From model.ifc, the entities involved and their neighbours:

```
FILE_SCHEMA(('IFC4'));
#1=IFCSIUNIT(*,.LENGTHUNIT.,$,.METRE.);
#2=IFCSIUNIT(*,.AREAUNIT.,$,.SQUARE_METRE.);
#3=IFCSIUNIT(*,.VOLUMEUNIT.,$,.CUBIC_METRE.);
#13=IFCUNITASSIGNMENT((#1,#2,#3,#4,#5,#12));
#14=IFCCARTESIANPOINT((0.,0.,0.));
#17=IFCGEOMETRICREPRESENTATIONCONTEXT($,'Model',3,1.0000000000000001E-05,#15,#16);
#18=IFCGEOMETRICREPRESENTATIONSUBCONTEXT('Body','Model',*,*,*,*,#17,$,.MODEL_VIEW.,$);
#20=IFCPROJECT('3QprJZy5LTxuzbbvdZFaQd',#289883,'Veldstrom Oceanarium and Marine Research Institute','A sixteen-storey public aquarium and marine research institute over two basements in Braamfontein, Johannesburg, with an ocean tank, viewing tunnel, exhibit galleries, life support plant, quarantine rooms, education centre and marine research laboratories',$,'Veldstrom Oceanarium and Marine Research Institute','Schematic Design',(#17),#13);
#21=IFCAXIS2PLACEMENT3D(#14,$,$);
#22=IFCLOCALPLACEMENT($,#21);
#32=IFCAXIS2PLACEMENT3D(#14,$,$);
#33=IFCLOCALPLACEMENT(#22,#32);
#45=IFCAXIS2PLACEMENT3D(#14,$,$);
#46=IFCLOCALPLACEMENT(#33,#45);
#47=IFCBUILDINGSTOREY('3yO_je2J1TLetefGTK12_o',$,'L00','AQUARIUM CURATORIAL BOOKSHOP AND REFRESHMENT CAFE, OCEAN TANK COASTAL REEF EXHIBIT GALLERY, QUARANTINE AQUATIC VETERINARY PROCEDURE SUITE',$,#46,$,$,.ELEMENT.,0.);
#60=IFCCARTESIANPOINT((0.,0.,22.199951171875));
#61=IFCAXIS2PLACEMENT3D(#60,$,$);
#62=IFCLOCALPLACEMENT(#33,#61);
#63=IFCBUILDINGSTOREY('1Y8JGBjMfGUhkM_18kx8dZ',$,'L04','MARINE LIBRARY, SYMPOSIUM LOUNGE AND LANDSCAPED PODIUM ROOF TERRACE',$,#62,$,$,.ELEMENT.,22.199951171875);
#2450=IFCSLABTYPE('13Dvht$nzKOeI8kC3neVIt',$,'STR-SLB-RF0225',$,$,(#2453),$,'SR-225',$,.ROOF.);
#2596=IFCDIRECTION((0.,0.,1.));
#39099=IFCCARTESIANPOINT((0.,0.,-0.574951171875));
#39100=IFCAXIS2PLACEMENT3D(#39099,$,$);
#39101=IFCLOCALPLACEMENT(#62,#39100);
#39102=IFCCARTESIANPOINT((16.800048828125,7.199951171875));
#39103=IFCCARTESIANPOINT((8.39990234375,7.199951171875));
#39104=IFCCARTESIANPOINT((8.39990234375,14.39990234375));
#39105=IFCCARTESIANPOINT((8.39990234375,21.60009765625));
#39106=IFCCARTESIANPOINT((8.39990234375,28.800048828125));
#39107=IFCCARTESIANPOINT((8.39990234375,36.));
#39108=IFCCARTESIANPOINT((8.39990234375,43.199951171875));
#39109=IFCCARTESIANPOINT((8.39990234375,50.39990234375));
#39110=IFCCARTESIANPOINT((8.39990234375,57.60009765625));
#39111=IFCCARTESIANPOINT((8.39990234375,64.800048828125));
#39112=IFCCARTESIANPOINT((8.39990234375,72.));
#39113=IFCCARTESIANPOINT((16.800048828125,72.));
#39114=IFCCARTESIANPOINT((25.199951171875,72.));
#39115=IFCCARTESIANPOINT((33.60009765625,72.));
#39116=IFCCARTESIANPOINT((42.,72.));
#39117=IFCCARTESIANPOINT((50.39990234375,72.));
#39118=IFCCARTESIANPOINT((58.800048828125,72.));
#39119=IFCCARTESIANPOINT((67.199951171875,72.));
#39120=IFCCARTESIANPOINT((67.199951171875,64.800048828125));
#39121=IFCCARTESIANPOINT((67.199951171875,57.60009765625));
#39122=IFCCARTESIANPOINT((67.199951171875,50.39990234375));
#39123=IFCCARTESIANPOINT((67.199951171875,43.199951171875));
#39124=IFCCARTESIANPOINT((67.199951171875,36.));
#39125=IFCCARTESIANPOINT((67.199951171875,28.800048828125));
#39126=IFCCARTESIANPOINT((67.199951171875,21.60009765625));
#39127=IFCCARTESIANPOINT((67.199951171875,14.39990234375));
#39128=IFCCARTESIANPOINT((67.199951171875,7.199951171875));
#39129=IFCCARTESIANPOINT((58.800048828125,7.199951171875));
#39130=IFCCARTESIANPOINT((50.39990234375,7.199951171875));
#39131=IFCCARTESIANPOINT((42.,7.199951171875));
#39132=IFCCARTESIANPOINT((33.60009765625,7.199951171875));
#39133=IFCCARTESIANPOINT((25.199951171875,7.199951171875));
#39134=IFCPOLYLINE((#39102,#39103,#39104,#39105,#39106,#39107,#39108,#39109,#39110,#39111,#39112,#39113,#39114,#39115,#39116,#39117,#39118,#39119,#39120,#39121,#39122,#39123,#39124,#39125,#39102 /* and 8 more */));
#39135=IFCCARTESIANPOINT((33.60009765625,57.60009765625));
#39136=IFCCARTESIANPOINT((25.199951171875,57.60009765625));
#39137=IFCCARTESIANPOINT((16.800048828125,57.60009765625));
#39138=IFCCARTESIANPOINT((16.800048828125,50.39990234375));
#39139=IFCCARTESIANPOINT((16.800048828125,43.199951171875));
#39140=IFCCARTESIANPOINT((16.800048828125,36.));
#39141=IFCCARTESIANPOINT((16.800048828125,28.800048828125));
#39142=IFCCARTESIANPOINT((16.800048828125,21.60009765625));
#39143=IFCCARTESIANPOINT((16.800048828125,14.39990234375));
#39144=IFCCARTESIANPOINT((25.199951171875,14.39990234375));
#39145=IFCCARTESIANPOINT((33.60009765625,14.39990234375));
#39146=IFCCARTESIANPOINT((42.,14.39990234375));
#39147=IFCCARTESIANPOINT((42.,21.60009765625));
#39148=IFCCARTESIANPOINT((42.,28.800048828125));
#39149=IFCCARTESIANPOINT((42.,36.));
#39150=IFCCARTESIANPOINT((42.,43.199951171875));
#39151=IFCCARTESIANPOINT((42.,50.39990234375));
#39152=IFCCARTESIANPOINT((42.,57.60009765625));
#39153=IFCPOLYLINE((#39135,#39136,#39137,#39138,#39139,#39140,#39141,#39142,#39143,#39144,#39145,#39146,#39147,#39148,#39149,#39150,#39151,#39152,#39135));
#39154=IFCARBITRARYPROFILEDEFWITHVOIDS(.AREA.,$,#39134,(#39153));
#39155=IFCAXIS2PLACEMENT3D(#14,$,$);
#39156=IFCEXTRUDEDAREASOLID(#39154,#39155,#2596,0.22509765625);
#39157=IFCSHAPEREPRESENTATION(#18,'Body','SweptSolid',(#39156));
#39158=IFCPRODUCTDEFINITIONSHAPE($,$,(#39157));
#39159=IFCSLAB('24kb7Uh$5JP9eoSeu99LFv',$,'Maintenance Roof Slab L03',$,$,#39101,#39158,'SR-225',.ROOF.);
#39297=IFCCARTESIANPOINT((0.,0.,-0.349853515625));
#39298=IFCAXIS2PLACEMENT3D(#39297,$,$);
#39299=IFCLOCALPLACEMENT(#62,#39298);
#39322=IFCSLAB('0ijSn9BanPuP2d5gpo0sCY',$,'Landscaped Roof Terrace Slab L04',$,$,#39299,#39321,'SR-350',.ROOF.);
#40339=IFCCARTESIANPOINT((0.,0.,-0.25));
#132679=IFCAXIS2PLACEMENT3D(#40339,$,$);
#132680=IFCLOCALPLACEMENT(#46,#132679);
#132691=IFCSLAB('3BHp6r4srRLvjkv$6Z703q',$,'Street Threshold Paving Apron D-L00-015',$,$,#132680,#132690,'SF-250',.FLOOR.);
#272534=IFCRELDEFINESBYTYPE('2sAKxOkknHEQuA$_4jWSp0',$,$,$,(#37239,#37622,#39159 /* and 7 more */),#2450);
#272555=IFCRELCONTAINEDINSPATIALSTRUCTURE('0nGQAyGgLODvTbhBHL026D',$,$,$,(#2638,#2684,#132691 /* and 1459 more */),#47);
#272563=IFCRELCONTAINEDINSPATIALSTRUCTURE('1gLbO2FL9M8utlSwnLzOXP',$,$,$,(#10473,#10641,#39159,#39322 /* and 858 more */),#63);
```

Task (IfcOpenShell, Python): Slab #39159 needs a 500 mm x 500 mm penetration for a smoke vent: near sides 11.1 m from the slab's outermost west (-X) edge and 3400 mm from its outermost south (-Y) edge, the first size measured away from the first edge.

```python
import numpy as np
import ifcopenshell
import ifcopenshell.api.feature
import ifcopenshell.api.geometry
import ifcopenshell.api.root
import ifcopenshell.geom
import ifcopenshell.util.placement
import ifcopenshell.util.representation
import ifcopenshell.util.shape
import ifcopenshell.util.unit

model = ifcopenshell.open("model.ifc")
unit_scale = ifcopenshell.util.unit.calculate_unit_scale(model)
settings = ifcopenshell.geom.settings()


def volume(element):
    """Net volume in cubic metres, openings subtracted."""
    shape = ifcopenshell.geom.create_shape(settings, element)
    return ifcopenshell.util.shape.get_volume(shape.geometry)


slab = model.by_guid("24kb7Uh$5JP9eoSeu99LFv")
before = volume(slab)

# Extent in the slab's own axes, in metres. The edges named are its -X and -Y sides.
slab_shape = ifcopenshell.geom.create_shape(settings, slab)
vertices = ifcopenshell.util.shape.get_vertices(slab_shape.geometry)
x_min, y_min, bottom = vertices.min(axis=0)
top = vertices[:, 2].max()

opening = ifcopenshell.api.root.create_entity(model, ifc_class="IfcOpeningElement", name="Smoke vent opening", predefined_type="OPENING")
context = ifcopenshell.util.representation.get_context(model, "Model", "Body", "MODEL_VIEW")
width, depth = 0.5, 0.5
outline = [(0.0, 0.0), (width, 0.0), (width, depth), (0.0, depth), (0.0, 0.0)]
# Overshoot both faces by 50 mm so the cut is clean.
shape = ifcopenshell.api.geometry.add_slab_representation(
    model, context=context, depth=top - bottom + 0.1, polyline=outline
)
ifcopenshell.api.geometry.assign_representation(model, product=opening, representation=shape)

matrix = ifcopenshell.util.placement.get_local_placement(slab.ObjectPlacement)
matrix[:, 3] = matrix @ np.append(np.array([x_min + 11.1, y_min + 3.4, bottom - 0.05]) / unit_scale, 1.0)
ifcopenshell.api.geometry.edit_object_placement(model, product=opening, matrix=matrix, is_si=False)
ifcopenshell.api.feature.add_feature(model, feature=opening, element=slab)

after = volume(slab)

print(f"slab volume {before:.3f} -> {after:.3f} m3")

model.write("model_v2.ifc")
```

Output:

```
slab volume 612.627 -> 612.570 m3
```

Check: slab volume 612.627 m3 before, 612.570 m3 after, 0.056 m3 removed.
